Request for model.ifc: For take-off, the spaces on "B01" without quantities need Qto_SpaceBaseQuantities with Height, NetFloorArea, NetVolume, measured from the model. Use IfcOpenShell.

First a look at what the model holds.

```python
import ifcopenshell
import ifcopenshell.util.element
import ifcopenshell.util.unit

model = ifcopenshell.open("model.ifc")
print(model.schema)
for unit_type in ("LENGTHUNIT", "AREAUNIT", "VOLUMEUNIT"):
    print(unit_type, ifcopenshell.util.unit.calculate_unit_scale(model, unit_type))
storey = next(s for s in model.by_type("IfcBuildingStorey") if s.Name == "B01")
spaces = [e for e in ifcopenshell.util.element.get_decomposition(storey) if e.is_a("IfcSpace")]
for e in sorted(spaces, key=lambda e: e.id()):
    print(e.id(), e.is_a(), e.Name, list(ifcopenshell.util.element.get_psets(e, qtos_only=True)), sep=" | ")
```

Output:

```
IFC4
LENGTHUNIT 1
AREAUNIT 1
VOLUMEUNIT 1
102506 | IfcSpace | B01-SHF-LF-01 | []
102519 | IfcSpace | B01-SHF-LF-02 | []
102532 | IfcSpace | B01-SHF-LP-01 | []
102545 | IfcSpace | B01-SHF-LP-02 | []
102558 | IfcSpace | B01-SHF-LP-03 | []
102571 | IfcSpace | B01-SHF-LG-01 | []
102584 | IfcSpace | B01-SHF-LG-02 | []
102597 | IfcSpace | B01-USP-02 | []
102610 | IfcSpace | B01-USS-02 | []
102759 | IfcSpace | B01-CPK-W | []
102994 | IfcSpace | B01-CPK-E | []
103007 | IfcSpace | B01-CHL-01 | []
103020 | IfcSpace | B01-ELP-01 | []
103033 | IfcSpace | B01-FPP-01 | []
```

```python
import ifcopenshell
import ifcopenshell.api.pset
import ifcopenshell.geom
import ifcopenshell.util.element
import ifcopenshell.util.shape
import ifcopenshell.util.unit

model = ifcopenshell.open("model.ifc")
unit_scale = ifcopenshell.util.unit.calculate_unit_scale(model)
area_scale = ifcopenshell.util.unit.calculate_unit_scale(model, "AREAUNIT")
volume_scale = ifcopenshell.util.unit.calculate_unit_scale(model, "VOLUMEUNIT")
settings = ifcopenshell.geom.settings()

storey = next(s for s in model.by_type("IfcBuildingStorey") if s.Name == "B01")
spaces = [e for e in ifcopenshell.util.element.get_decomposition(storey) if e.is_a("IfcSpace")]

for e in sorted(spaces, key=lambda e: e.id()):
    if ifcopenshell.util.element.get_psets(e, qtos_only=True, should_inherit=False):
        continue
    # Geometry comes back in metres, in the element's own axes.
    shape = ifcopenshell.geom.create_shape(settings, e)
    values = {
        "Height": ifcopenshell.util.shape.get_z(shape.geometry) / unit_scale,
        "NetFloorArea": ifcopenshell.util.shape.get_footprint_area(shape.geometry) / area_scale,
        "NetVolume": ifcopenshell.util.shape.get_volume(shape.geometry) / volume_scale,
    }
    qto = ifcopenshell.api.pset.add_qto(model, product=e, name="Qto_SpaceBaseQuantities")
    ifcopenshell.api.pset.edit_qto(model, qto=qto, properties=values)
    print(e.id(), {k: round(v, 3) for k, v in values.items()})

model.write("model_edited.ifc")
```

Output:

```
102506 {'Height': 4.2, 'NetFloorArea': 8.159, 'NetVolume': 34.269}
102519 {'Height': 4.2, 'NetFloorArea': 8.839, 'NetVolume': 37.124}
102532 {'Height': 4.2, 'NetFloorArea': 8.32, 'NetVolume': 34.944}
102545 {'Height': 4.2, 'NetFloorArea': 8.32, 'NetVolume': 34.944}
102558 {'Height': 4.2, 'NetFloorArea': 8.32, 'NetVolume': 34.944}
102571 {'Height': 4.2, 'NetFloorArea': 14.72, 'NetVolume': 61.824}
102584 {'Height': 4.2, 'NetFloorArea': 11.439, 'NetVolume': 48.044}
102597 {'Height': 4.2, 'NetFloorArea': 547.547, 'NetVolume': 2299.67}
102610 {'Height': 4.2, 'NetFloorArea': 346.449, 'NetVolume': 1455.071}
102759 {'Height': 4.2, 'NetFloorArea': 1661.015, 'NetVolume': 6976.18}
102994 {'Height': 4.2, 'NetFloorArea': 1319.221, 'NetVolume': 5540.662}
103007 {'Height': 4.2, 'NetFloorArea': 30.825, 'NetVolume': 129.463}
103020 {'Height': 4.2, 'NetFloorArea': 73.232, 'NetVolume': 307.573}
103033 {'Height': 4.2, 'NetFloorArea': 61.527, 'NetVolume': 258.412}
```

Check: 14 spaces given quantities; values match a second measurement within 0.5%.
